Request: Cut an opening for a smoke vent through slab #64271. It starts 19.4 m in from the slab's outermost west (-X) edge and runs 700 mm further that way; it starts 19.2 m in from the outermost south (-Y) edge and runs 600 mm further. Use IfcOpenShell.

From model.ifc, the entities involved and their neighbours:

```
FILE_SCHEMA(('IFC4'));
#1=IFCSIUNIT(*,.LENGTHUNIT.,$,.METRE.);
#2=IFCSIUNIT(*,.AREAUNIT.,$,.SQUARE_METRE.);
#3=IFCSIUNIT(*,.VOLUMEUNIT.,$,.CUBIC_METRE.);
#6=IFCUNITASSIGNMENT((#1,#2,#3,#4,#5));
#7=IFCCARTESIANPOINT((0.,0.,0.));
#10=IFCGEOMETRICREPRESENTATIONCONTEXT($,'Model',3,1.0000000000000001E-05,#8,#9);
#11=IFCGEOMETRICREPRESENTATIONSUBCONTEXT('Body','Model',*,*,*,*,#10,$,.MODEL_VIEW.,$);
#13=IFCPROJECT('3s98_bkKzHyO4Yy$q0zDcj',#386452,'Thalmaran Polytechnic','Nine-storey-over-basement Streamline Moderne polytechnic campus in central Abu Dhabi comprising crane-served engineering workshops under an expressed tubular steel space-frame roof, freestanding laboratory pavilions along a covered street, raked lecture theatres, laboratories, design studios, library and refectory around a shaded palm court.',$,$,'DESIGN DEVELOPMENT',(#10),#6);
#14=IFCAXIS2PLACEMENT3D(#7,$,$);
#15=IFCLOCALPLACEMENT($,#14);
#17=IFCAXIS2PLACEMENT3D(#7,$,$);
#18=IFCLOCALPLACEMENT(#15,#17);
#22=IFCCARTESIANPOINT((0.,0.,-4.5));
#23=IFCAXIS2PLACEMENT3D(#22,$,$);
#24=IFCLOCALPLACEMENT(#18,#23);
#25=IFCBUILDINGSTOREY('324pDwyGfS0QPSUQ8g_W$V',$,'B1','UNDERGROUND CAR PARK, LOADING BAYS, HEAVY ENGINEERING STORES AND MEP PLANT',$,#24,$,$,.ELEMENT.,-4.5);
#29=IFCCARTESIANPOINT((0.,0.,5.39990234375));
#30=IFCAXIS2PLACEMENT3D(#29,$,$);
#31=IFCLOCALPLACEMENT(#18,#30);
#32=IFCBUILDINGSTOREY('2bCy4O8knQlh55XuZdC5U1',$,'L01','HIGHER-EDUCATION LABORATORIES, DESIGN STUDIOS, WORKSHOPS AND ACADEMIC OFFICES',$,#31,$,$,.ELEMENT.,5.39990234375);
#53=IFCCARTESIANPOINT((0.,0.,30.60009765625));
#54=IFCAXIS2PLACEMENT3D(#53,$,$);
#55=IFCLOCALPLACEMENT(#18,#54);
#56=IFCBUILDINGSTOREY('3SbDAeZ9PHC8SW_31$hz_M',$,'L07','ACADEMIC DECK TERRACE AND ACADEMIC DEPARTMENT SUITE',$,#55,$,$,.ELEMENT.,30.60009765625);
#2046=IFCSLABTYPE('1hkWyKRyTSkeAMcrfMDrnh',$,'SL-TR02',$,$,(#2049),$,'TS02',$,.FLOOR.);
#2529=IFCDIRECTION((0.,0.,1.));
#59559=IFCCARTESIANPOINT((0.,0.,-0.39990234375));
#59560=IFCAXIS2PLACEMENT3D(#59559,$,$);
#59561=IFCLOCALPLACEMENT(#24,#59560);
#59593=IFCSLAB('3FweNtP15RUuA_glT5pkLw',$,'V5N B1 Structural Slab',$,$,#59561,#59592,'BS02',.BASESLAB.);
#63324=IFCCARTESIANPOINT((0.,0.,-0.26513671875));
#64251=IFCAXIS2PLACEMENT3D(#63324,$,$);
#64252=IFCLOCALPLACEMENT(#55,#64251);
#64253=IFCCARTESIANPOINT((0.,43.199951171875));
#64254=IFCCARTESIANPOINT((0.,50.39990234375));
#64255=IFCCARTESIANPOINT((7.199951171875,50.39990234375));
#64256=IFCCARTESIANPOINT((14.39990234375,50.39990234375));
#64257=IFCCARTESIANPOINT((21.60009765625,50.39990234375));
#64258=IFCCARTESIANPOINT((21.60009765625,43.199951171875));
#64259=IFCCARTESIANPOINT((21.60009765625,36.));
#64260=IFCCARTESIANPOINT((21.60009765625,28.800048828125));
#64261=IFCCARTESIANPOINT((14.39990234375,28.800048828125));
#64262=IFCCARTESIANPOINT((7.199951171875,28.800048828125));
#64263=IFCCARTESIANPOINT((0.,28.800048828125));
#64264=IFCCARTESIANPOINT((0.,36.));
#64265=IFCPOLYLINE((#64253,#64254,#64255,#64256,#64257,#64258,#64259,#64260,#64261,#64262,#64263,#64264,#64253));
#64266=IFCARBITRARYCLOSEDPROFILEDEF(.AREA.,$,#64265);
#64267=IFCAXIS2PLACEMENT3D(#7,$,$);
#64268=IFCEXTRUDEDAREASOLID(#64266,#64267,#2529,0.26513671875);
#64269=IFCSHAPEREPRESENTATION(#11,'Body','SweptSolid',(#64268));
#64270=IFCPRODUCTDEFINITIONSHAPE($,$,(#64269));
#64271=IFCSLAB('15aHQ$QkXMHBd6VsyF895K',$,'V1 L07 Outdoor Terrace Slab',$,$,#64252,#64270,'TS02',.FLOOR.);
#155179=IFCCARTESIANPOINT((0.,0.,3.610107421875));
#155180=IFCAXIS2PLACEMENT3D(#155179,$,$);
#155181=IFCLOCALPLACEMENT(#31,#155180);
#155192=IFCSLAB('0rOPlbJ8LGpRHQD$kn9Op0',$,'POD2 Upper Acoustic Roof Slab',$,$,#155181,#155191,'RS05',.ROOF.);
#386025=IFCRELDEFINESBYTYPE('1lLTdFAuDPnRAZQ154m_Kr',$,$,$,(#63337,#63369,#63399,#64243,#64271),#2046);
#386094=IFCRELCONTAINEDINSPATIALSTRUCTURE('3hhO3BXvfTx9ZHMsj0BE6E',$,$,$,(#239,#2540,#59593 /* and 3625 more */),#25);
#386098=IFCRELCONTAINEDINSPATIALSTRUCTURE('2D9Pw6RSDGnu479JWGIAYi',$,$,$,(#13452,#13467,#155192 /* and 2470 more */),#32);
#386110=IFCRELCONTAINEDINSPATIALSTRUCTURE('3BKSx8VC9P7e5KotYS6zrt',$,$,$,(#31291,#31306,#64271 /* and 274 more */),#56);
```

```python
import numpy as np
import ifcopenshell
import ifcopenshell.api.feature
import ifcopenshell.api.geometry
import ifcopenshell.api.root
import ifcopenshell.geom
import ifcopenshell.util.placement
import ifcopenshell.util.representation
import ifcopenshell.util.shape
import ifcopenshell.util.unit

model = ifcopenshell.open("model.ifc")
unit_scale = ifcopenshell.util.unit.calculate_unit_scale(model)
settings = ifcopenshell.geom.settings()


def volume(element):
    """Net volume in cubic metres, openings subtracted."""
    shape = ifcopenshell.geom.create_shape(settings, element)
    return ifcopenshell.util.shape.get_volume(shape.geometry)


slab = model.by_id(64271)
before = volume(slab)

# Extent in the slab's own axes, in metres. The edges named are its -X and -Y sides.
slab_shape = ifcopenshell.geom.create_shape(settings, slab)
vertices = ifcopenshell.util.shape.get_vertices(slab_shape.geometry)
x_min, y_min, bottom = vertices.min(axis=0)
top = vertices[:, 2].max()

opening = ifcopenshell.api.root.create_entity(model, ifc_class="IfcOpeningElement", name="Smoke vent opening", predefined_type="OPENING")
context = ifcopenshell.util.representation.get_context(model, "Model", "Body", "MODEL_VIEW")
width, depth = 0.7, 0.6
outline = [(0.0, 0.0), (width, 0.0), (width, depth), (0.0, depth), (0.0, 0.0)]
# Overshoot both faces by 50 mm so the cut is clean.
shape = ifcopenshell.api.geometry.add_slab_representation(
    model, context=context, depth=top - bottom + 0.1, polyline=outline
)
ifcopenshell.api.geometry.assign_representation(model, product=opening, representation=shape)

matrix = ifcopenshell.util.placement.get_local_placement(slab.ObjectPlacement)
matrix[:, 3] = matrix @ np.append(np.array([x_min + 19.4, y_min + 19.2, bottom - 0.05]) / unit_scale, 1.0)
ifcopenshell.api.geometry.edit_object_placement(model, product=opening, matrix=matrix, is_si=False)
ifcopenshell.api.feature.add_feature(model, feature=opening, element=slab)

after = volume(slab)

print(f"slab volume {before:.3f} -> {after:.3f} m3")

model.write("model_v2.ifc")
```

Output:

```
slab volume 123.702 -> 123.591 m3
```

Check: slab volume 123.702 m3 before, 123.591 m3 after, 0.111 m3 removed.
